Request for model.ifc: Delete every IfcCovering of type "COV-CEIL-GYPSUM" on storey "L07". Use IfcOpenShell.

First a look at what the model holds.

```python
import ifcopenshell
import ifcopenshell.util.element

model = ifcopenshell.open("model.ifc")
print(model.schema)
storey = next(s for s in model.by_type("IfcBuildingStorey") if s.Name == "L07")
coverings = [e for e in ifcopenshell.util.element.get_decomposition(storey) if e.is_a("IfcCovering")]
seen = {}
for e in coverings:
    element_type = ifcopenshell.util.element.get_type(e)
    name = element_type.Name if element_type not in (None, e) else None
    seen[name] = seen.get(name, 0) + 1
for name, count in sorted(seen.items(), key=str):
    print(count, "x", name)
```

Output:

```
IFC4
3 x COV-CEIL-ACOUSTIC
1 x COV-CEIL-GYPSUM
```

```python
import ifcopenshell
import ifcopenshell.api.root
import ifcopenshell.util.element

model = ifcopenshell.open("model.ifc")

storey = next(s for s in model.by_type("IfcBuildingStorey") if s.Name == "L07")
coverings = [e for e in ifcopenshell.util.element.get_decomposition(storey) if e.is_a("IfcCovering")]
targets = [e for e in coverings if (t := ifcopenshell.util.element.get_type(e)) not in (None, e) and t.Name == "COV-CEIL-GYPSUM"]

for e in targets:
    ifcopenshell.api.root.remove_product(model, product=e)
print(len(targets), "removed")

model.write("model_rev.ifc")
```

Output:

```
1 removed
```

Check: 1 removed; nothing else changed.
